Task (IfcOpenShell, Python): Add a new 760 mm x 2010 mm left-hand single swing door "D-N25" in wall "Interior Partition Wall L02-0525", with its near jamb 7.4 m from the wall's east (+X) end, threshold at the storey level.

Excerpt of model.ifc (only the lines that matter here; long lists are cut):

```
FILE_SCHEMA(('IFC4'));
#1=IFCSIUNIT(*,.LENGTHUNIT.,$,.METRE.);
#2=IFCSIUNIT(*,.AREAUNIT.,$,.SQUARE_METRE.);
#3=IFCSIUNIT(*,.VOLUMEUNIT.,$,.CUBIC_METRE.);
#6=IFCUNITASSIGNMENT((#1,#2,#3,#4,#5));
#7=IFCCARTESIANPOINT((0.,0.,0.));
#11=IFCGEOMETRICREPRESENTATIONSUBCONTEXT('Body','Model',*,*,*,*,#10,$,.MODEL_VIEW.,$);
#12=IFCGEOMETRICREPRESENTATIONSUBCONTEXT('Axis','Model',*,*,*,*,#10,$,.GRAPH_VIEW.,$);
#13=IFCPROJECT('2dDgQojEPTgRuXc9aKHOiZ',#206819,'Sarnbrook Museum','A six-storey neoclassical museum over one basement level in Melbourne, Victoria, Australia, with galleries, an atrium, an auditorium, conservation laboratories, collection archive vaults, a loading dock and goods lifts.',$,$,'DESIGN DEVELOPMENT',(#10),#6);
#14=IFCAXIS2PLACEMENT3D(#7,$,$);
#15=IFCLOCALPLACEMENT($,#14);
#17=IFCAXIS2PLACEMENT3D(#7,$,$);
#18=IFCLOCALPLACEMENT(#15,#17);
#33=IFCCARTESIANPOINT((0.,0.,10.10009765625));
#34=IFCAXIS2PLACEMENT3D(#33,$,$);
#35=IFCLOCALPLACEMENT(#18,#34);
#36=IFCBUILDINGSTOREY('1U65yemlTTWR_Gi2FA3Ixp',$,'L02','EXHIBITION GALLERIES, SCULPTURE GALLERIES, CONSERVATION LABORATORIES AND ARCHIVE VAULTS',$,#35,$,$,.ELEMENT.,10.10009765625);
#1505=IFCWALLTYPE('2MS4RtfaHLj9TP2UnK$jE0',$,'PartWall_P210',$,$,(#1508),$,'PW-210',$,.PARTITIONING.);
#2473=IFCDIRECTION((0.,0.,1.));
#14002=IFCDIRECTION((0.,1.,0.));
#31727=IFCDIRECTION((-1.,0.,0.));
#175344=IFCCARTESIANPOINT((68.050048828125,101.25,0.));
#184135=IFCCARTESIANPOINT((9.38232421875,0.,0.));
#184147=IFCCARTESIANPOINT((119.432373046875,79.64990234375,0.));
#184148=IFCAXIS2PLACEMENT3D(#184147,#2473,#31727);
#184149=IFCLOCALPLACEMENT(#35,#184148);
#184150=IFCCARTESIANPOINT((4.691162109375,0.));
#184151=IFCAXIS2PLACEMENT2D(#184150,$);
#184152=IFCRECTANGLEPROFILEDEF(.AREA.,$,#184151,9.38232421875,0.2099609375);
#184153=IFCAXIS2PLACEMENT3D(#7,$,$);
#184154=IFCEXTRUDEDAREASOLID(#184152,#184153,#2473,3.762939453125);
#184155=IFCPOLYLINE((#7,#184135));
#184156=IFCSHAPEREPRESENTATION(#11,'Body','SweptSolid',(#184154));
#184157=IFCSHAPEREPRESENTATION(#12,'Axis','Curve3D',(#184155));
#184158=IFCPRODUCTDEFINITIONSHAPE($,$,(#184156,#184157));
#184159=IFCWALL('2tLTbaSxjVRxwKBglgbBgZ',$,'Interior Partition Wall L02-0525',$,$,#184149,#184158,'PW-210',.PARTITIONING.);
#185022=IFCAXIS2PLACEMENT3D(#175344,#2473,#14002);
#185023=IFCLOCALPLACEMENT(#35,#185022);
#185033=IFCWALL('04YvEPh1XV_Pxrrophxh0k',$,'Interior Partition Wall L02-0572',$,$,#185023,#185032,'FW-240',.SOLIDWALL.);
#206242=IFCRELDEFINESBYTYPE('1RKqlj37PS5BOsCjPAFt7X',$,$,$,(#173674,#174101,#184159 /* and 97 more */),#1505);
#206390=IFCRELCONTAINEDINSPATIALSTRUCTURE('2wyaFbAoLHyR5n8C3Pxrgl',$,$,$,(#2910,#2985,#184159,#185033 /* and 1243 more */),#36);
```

```python
import numpy as np
import ifcopenshell
import ifcopenshell.api.feature
import ifcopenshell.api.geometry
import ifcopenshell.api.root
import ifcopenshell.api.spatial
import ifcopenshell.geom
import ifcopenshell.util.element
import ifcopenshell.util.placement
import ifcopenshell.util.representation
import ifcopenshell.util.shape
import ifcopenshell.util.unit

model = ifcopenshell.open("model.ifc")
unit_scale = ifcopenshell.util.unit.calculate_unit_scale(model)
settings = ifcopenshell.geom.settings()


def volume(element):
    """Net volume in cubic metres, openings subtracted."""
    shape = ifcopenshell.geom.create_shape(settings, element)
    return ifcopenshell.util.shape.get_volume(shape.geometry)


wall = model.by_guid("2tLTbaSxjVRxwKBglgbBgZ")
storey = ifcopenshell.util.element.get_container(wall, ifc_class="IfcBuildingStorey")
context = ifcopenshell.util.representation.get_context(model, "Model", "Body", "MODEL_VIEW")
before = volume(wall)

width, height, from_end, sill = 0.76, 2.01, 7.4, 0.0  # metres

# The wall runs along its own X axis, and the end named is its -X end.
wall_shape = ifcopenshell.geom.create_shape(settings, wall)
x, y, z = ifcopenshell.util.shape.get_vertices(wall_shape.geometry).T
start = x.min() + from_end
face, thickness = float(y.min()), float(y.max() - y.min())
wall_matrix = ifcopenshell.util.placement.get_local_placement(wall.ObjectPlacement)
level = ifcopenshell.util.placement.get_local_placement(storey.ObjectPlacement)[2, 3]


def in_wall(x, y):
    """Placement at x, y metres in the wall's axes, at sill height."""
    matrix = wall_matrix.copy()
    matrix[:, 3] = wall_matrix @ np.array([x / unit_scale, y / unit_scale, 0.0, 1.0])
    matrix[2, 3] = level + sill / unit_scale
    return matrix


# Opening: a box that overshoots both wall faces by 50 mm.
opening = ifcopenshell.api.root.create_entity(model, ifc_class="IfcOpeningElement", predefined_type="OPENING")
box = ifcopenshell.api.geometry.add_wall_representation(
    model, context=context, length=width, height=height, thickness=thickness + 0.1
)
ifcopenshell.api.geometry.assign_representation(model, product=opening, representation=box)
ifcopenshell.api.geometry.edit_object_placement(model, product=opening, matrix=in_wall(start, face - 0.05), is_si=False)
ifcopenshell.api.feature.add_feature(model, feature=opening, element=wall)

door = ifcopenshell.api.root.create_entity(model, ifc_class="IfcDoor", name="D-N25", predefined_type="DOOR")
door.OverallWidth, door.OverallHeight = width / unit_scale, height / unit_scale
door.OperationType = "SINGLE_SWING_LEFT"
body = ifcopenshell.api.geometry.add_door_representation(
    model,
    context=context,
    overall_width=door.OverallWidth,
    overall_height=door.OverallHeight,
    operation_type="SINGLE_SWING_LEFT",
    lining_properties={"LiningDepth": thickness / unit_scale, "ThresholdDepth": thickness / unit_scale},
)
ifcopenshell.api.geometry.assign_representation(model, product=door, representation=body)
ifcopenshell.api.spatial.assign_container(model, products=[door], relating_structure=storey)
ifcopenshell.api.feature.add_filling(model, opening=opening, element=door)

# The lining spans the wall, so the door starts at the wall face.
ifcopenshell.api.geometry.edit_object_placement(model, product=door, matrix=in_wall(start, face), is_si=False)

after = volume(wall)

print(f"wall volume {before:.3f} -> {after:.3f} m3")

model.write("model_updated.ifc")
```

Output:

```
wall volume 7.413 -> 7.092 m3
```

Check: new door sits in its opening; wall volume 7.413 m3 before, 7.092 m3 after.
